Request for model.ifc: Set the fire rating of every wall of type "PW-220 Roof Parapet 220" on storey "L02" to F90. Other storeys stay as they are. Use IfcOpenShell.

First a look at what the model holds.

```python
import ifcopenshell
import ifcopenshell.util.element

model = ifcopenshell.open("model.ifc")
print(model.schema)
storey = next(s for s in model.by_type("IfcBuildingStorey") if s.Name == "L02")
walls = [e for e in ifcopenshell.util.element.get_decomposition(storey) if e.is_a("IfcWall")]
seen = {}
for e in walls:
    element_type = ifcopenshell.util.element.get_type(e)
    key = (element_type.Name if element_type != e and element_type else None, ifcopenshell.util.element.get_pset(e, "Pset_WallCommon", "FireRating"))
    seen[key] = seen.get(key, 0) + 1
for (name, value), count in sorted(seen.items(), key=str):
    print(count, "x", name, "|", value)
```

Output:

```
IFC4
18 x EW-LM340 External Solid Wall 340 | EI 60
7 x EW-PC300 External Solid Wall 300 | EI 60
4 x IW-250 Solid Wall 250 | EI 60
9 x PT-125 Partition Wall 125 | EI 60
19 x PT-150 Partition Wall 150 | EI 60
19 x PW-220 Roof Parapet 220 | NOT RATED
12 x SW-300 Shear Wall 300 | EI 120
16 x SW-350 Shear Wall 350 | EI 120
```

```python
import ifcopenshell
import ifcopenshell.api.pset
import ifcopenshell.util.element

model = ifcopenshell.open("model.ifc")

storey = next(s for s in model.by_type("IfcBuildingStorey") if s.Name == "L02")
walls = [e for e in ifcopenshell.util.element.get_decomposition(storey) if e.is_a("IfcWall")]

count = 0
for e in walls:
    element_type = ifcopenshell.util.element.get_type(e)
    if element_type in (None, e) or element_type.Name != "PW-220 Roof Parapet 220":
        continue
    # add_pset returns the element's existing set when there is one.
    pset = ifcopenshell.api.pset.add_pset(model, product=e, name="Pset_WallCommon")
    ifcopenshell.api.pset.edit_pset(model, pset=pset, properties={"FireRating": "F90"})
    count += 1

print(count, "walls updated")

model.write("model_v2.ifc")
```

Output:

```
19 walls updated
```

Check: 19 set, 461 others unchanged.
